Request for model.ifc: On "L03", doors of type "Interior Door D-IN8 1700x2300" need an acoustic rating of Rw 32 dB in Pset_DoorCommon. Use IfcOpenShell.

First a look at what the model holds.

```python
import ifcopenshell
import ifcopenshell.util.element

model = ifcopenshell.open("model.ifc")
print(model.schema)
storey = next(s for s in model.by_type("IfcBuildingStorey") if s.Name == "L03")
doors = [e for e in ifcopenshell.util.element.get_decomposition(storey) if e.is_a("IfcDoor")]
seen = {}
for e in doors:
    element_type = ifcopenshell.util.element.get_type(e)
    key = (element_type.Name if element_type != e and element_type else None, ifcopenshell.util.element.get_pset(e, "Pset_DoorCommon", "AcousticRating"))
    seen[key] = seen.get(key, 0) + 1
for (name, value), count in sorted(seen.items(), key=str):
    print(count, "x", name, "|", value)
```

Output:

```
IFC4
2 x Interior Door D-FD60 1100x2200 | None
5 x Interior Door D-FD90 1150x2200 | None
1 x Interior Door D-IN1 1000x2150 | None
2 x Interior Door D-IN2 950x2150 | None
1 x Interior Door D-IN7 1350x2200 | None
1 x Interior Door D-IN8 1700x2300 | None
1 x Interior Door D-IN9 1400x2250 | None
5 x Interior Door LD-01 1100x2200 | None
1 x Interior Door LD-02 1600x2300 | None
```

```python
import ifcopenshell
import ifcopenshell.api.pset
import ifcopenshell.util.element

model = ifcopenshell.open("model.ifc")

storey = next(s for s in model.by_type("IfcBuildingStorey") if s.Name == "L03")
doors = [e for e in ifcopenshell.util.element.get_decomposition(storey) if e.is_a("IfcDoor")]

count = 0
for e in doors:
    element_type = ifcopenshell.util.element.get_type(e)
    if element_type in (None, e) or element_type.Name != "Interior Door D-IN8 1700x2300":
        continue
    # add_pset returns the element's existing set when there is one.
    pset = ifcopenshell.api.pset.add_pset(model, product=e, name="Pset_DoorCommon")
    ifcopenshell.api.pset.edit_pset(model, pset=pset, properties={"AcousticRating": "Rw 32 dB"})
    count += 1

print(count, "doors updated")

model.write("model_v2.ifc")
```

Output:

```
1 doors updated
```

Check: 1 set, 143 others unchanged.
